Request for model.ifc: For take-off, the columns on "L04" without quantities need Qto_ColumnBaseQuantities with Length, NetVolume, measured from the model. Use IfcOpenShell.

First a look at what the model holds.

```python
import ifcopenshell
import ifcopenshell.util.element
import ifcopenshell.util.unit

model = ifcopenshell.open("model.ifc")
print(model.schema)
for unit_type in ("LENGTHUNIT", "AREAUNIT", "VOLUMEUNIT"):
    print(unit_type, ifcopenshell.util.unit.calculate_unit_scale(model, unit_type))
storey = next(s for s in model.by_type("IfcBuildingStorey") if s.Name == "L04")
columns = [e for e in ifcopenshell.util.element.get_decomposition(storey) if e.is_a("IfcColumn")]
for e in sorted(columns, key=lambda e: e.id()):
    print(e.id(), e.is_a(), e.Name, list(ifcopenshell.util.element.get_psets(e, qtos_only=True)), sep=" | ")
```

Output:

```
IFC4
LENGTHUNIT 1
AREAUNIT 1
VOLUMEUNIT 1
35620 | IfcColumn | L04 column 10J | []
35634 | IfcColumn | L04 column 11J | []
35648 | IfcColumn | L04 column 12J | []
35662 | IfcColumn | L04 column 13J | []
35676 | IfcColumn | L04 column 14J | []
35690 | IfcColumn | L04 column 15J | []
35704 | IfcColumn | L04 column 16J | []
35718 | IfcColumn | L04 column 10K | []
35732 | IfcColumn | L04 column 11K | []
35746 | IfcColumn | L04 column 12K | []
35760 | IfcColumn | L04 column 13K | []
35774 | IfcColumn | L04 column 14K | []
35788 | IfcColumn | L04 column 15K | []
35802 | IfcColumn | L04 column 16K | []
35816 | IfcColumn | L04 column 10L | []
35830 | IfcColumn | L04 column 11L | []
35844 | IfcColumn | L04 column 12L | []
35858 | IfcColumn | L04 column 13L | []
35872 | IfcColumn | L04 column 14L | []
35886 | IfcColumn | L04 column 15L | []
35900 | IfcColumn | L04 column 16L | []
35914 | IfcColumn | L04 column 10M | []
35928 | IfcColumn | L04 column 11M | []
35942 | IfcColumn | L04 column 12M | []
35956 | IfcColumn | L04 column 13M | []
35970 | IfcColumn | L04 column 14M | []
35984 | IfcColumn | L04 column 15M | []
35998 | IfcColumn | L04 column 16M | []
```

```python
import ifcopenshell
import ifcopenshell.api.pset
import ifcopenshell.geom
import ifcopenshell.util.element
import ifcopenshell.util.shape
import ifcopenshell.util.unit

model = ifcopenshell.open("model.ifc")
unit_scale = ifcopenshell.util.unit.calculate_unit_scale(model)
volume_scale = ifcopenshell.util.unit.calculate_unit_scale(model, "VOLUMEUNIT")
settings = ifcopenshell.geom.settings()

storey = next(s for s in model.by_type("IfcBuildingStorey") if s.Name == "L04")
columns = [e for e in ifcopenshell.util.element.get_decomposition(storey) if e.is_a("IfcColumn")]

for e in sorted(columns, key=lambda e: e.id()):
    if ifcopenshell.util.element.get_psets(e, qtos_only=True, should_inherit=False):
        continue
    # Geometry comes back in metres, in the element's own axes.
    shape = ifcopenshell.geom.create_shape(settings, e)
    values = {
        "Length": ifcopenshell.util.shape.get_z(shape.geometry) / unit_scale,
        "NetVolume": ifcopenshell.util.shape.get_volume(shape.geometry) / volume_scale,
    }
    qto = ifcopenshell.api.pset.add_qto(model, product=e, name="Qto_ColumnBaseQuantities")
    ifcopenshell.api.pset.edit_qto(model, qto=qto, properties=values)
    print(e.id(), {k: round(v, 3) for k, v in values.items()})

model.write("model_rev.ifc")
```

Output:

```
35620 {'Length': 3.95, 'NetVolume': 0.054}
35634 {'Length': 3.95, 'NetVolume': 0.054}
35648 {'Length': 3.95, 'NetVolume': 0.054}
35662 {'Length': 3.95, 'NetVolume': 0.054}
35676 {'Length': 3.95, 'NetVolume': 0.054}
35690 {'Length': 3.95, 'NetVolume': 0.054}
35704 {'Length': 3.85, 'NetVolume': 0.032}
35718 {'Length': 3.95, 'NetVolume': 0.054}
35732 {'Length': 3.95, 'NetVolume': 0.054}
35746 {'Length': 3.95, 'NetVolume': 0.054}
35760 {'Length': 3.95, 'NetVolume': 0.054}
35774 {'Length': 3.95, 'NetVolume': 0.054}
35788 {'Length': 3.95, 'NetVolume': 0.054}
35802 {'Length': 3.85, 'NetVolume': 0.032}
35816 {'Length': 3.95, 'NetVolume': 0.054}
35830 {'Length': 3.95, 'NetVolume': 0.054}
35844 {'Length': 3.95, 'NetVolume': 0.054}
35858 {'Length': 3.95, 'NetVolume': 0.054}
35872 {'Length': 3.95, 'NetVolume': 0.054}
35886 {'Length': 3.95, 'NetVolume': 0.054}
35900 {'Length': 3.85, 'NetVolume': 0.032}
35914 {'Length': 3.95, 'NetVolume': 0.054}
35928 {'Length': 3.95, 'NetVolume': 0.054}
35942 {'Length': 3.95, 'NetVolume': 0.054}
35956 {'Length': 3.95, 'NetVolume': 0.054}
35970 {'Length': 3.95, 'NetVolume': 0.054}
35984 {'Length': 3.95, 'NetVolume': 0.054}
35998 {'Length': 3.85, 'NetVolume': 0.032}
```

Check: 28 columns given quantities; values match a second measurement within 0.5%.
